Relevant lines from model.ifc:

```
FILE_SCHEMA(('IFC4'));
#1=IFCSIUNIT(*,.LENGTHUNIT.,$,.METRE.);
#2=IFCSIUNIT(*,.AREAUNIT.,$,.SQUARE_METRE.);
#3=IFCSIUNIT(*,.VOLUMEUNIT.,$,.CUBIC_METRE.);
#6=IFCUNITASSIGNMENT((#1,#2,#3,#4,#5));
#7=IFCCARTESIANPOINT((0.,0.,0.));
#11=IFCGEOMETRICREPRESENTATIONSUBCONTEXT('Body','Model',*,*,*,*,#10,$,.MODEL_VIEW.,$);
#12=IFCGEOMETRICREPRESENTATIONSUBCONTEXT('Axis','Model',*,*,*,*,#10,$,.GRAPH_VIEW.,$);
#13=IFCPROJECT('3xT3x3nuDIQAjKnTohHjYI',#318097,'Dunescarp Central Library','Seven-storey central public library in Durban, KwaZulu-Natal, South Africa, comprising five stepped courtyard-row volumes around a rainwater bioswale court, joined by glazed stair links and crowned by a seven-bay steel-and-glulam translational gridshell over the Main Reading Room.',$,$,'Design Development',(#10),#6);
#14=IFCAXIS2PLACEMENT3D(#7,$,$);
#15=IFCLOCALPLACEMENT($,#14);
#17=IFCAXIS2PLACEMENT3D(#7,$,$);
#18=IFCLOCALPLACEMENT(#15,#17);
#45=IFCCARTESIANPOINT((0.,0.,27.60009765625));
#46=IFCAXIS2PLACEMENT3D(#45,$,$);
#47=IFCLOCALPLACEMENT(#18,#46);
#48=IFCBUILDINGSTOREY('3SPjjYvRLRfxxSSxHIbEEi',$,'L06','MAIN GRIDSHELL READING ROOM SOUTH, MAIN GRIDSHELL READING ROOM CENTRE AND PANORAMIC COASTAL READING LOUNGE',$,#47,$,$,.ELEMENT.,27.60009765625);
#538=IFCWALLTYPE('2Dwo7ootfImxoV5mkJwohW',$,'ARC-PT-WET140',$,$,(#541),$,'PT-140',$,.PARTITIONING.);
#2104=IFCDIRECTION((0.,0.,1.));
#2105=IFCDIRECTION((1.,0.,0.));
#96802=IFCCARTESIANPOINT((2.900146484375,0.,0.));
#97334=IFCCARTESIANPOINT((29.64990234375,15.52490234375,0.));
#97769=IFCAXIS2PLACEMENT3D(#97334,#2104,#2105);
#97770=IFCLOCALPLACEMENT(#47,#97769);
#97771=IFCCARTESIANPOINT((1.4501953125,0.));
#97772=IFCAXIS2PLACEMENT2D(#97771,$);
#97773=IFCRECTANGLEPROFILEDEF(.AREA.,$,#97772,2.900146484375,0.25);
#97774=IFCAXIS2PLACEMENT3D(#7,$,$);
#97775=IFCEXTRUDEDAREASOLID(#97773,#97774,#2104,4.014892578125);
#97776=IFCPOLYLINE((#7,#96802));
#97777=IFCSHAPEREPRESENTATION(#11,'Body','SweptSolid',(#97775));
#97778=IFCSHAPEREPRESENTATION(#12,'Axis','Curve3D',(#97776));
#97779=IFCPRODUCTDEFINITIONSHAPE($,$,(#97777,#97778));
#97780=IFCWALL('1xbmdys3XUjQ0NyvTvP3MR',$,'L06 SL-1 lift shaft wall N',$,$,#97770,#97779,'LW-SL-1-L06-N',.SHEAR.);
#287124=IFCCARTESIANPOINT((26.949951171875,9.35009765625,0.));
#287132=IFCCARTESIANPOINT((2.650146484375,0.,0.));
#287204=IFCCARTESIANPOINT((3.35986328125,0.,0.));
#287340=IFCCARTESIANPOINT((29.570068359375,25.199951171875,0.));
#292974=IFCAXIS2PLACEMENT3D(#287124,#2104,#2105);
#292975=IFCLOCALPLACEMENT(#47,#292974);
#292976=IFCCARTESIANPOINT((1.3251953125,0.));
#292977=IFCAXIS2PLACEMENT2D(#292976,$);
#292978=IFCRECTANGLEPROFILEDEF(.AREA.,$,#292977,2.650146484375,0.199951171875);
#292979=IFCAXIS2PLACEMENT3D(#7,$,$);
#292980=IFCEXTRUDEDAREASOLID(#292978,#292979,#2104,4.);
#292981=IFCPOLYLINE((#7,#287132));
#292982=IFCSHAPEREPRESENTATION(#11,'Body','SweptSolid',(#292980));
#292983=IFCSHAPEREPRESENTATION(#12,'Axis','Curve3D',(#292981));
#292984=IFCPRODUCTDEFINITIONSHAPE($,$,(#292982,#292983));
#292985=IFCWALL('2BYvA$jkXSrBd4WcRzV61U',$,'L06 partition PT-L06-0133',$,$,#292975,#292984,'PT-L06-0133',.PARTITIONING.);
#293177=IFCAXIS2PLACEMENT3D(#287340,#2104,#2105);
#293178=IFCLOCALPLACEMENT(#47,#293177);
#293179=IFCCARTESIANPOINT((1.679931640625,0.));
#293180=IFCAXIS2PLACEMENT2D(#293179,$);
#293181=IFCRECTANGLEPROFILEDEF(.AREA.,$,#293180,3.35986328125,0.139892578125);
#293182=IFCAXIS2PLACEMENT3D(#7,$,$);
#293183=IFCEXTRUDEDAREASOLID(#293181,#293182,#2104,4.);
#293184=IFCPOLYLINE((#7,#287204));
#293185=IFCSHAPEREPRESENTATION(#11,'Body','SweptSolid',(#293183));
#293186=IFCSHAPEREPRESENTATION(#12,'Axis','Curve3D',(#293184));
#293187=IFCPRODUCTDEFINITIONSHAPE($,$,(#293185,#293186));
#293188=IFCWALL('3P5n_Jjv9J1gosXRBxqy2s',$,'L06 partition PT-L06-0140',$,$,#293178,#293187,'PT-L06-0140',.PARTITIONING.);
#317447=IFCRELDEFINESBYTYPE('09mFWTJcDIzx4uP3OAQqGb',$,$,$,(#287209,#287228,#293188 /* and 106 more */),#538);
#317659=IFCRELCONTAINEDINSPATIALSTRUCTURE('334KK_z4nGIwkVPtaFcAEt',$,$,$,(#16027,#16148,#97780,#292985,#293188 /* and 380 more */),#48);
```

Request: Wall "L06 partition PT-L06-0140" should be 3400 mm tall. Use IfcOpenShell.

```python
import ifcopenshell
import ifcopenshell.geom
import ifcopenshell.util.representation
import ifcopenshell.util.shape
import ifcopenshell.util.unit

model = ifcopenshell.open("model.ifc")
unit_scale = ifcopenshell.util.unit.calculate_unit_scale(model)
settings = ifcopenshell.geom.settings()


def volume(element):
    """Net volume in cubic metres, openings subtracted."""
    shape = ifcopenshell.geom.create_shape(settings, element)
    return ifcopenshell.util.shape.get_volume(shape.geometry)


wall = model.by_guid("3P5n_Jjv9J1gosXRBxqy2s")
before = volume(wall)

body = ifcopenshell.util.representation.get_representation(wall, "Model", "Body")
solid = body.Items[0]
old_height = solid.Depth
solid.Depth = 3.4 / unit_scale
after = volume(wall)

print(f"height {old_height:g} -> {solid.Depth:g}, volume {before:.3f} -> {after:.3f} m3")

model.write("model-out.ifc")
```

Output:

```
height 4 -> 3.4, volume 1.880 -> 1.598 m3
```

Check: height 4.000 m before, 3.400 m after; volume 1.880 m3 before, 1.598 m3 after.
